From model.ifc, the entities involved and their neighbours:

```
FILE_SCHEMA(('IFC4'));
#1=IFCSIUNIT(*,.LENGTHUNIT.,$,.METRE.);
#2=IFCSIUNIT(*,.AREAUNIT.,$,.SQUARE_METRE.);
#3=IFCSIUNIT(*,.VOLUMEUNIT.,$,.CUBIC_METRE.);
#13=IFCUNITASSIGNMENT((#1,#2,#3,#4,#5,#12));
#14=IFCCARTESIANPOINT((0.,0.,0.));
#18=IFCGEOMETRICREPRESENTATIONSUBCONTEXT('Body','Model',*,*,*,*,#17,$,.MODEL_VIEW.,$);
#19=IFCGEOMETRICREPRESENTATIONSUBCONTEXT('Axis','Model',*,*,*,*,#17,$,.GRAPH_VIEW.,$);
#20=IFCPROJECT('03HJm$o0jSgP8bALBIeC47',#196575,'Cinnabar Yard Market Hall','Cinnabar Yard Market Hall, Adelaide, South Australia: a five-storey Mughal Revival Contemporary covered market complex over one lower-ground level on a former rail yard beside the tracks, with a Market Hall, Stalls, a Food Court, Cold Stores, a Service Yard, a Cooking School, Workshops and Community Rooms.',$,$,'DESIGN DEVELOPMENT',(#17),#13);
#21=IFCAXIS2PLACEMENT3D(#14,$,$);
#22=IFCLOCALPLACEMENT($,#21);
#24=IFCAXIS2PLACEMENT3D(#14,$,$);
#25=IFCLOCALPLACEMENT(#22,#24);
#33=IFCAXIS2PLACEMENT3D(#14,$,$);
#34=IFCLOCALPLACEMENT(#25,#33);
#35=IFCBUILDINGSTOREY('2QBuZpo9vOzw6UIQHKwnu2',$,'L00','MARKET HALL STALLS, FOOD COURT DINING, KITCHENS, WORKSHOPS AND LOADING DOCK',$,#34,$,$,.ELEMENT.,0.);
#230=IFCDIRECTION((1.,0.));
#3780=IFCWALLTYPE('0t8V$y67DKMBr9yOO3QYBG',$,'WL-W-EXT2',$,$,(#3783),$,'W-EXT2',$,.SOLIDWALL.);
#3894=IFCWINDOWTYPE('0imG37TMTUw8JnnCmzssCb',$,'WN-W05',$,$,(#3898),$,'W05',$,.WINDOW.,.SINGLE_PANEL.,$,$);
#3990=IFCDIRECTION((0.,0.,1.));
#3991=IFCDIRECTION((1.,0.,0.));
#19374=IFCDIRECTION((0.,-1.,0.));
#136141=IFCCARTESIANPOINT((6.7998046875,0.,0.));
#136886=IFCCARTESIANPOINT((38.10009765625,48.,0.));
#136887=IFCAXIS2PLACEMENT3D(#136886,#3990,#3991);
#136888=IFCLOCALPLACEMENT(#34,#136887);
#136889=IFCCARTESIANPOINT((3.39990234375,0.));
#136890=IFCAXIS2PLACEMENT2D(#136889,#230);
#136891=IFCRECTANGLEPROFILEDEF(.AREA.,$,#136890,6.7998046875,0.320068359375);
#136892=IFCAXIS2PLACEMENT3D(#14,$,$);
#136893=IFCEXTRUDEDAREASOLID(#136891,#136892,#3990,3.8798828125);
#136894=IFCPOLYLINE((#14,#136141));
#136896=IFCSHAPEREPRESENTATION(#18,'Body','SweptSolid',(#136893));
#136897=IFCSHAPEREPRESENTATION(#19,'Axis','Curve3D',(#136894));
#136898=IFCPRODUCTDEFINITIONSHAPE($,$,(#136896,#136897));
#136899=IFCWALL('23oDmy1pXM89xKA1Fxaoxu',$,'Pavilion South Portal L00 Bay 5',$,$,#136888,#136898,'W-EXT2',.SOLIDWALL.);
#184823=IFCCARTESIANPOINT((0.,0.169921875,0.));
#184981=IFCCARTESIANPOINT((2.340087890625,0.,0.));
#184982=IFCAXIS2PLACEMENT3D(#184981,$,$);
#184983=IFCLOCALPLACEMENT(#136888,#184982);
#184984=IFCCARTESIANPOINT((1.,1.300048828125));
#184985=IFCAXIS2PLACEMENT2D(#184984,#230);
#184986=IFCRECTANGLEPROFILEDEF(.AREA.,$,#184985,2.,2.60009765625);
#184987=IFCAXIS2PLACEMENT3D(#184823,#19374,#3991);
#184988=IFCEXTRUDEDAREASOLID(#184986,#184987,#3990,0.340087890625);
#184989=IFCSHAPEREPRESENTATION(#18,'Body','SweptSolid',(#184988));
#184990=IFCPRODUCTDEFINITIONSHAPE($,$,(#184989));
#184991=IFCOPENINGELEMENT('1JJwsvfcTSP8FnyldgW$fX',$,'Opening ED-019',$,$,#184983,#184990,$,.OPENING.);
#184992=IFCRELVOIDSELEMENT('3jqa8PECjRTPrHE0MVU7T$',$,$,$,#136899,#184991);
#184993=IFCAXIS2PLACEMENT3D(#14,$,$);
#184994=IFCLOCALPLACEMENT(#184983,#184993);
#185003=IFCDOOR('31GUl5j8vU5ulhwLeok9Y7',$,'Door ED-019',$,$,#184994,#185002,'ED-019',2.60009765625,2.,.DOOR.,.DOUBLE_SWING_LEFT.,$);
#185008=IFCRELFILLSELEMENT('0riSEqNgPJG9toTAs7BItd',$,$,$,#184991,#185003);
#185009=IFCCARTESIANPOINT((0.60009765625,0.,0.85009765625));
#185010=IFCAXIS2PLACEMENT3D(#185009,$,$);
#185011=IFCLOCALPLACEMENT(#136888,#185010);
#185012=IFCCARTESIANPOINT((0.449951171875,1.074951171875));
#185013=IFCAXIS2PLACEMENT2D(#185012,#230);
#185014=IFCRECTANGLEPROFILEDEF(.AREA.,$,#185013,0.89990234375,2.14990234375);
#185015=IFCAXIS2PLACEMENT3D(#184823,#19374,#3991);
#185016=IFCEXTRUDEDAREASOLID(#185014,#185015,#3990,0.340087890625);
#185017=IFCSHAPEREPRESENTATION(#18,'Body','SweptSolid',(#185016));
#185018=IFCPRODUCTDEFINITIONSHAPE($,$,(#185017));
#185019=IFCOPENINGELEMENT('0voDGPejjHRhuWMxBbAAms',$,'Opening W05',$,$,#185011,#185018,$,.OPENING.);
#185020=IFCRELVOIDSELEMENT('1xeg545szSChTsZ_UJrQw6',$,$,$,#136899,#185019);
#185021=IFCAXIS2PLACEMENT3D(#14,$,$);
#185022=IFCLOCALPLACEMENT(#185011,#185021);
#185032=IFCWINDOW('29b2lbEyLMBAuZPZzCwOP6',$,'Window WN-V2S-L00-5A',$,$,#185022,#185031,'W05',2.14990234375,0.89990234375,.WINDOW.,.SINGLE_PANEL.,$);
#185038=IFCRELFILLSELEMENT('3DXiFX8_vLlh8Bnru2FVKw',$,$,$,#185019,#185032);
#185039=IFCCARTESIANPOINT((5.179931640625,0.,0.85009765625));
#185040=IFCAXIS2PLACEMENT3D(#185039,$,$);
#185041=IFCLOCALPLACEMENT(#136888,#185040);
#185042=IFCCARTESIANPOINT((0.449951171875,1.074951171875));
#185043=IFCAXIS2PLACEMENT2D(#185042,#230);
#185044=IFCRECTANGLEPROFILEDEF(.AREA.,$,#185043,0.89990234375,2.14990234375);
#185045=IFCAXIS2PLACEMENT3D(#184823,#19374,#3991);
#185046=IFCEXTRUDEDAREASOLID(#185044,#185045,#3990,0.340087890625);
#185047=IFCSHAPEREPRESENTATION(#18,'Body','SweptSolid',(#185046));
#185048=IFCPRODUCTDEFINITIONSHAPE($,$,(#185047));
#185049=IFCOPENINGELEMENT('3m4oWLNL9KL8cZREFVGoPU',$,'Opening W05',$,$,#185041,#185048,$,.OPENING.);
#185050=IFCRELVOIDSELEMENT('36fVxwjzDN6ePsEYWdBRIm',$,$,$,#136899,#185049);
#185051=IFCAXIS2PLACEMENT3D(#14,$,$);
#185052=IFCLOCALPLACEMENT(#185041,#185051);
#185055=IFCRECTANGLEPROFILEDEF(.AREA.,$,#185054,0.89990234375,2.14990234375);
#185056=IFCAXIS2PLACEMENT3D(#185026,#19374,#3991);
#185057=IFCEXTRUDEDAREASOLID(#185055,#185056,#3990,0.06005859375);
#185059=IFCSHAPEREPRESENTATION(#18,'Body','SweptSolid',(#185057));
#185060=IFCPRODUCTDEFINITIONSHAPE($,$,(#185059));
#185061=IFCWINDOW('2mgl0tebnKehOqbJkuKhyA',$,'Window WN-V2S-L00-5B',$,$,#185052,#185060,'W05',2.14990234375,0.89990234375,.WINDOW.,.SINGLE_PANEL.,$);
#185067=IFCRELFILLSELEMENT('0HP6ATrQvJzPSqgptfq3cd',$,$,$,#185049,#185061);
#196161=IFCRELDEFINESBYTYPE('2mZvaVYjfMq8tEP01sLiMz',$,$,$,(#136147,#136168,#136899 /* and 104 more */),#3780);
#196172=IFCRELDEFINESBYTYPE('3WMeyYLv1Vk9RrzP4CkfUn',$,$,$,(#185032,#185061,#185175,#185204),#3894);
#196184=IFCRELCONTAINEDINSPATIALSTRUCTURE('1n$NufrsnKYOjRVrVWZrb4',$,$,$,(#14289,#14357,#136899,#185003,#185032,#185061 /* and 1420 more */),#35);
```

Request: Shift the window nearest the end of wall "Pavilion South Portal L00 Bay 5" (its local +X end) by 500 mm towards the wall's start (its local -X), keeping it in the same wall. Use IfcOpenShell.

```python
import ifcopenshell
import ifcopenshell.api.geometry
import ifcopenshell.util.placement
import ifcopenshell.util.unit

model = ifcopenshell.open("model.ifc")
unit_scale = ifcopenshell.util.unit.calculate_unit_scale(model)

window = model.by_id(185061)
opening = window.FillsVoids[0].RelatingOpeningElement
wall = opening.VoidsElements[0].RelatingBuildingElement

wall_matrix = ifcopenshell.util.placement.get_local_placement(wall.ObjectPlacement)
shift = wall_matrix[:3, 0] * -0.5 / unit_scale
before = ifcopenshell.util.placement.get_local_placement(window.ObjectPlacement)[:3, 3].copy()

# The window is placed relative to its opening, so it follows when the opening moves.
matrix = ifcopenshell.util.placement.get_local_placement(opening.ObjectPlacement)
matrix[:3, 3] += shift
ifcopenshell.api.geometry.edit_object_placement(
    model, product=opening, matrix=matrix, is_si=False, should_transform_children=True
)

after = ifcopenshell.util.placement.get_local_placement(window.ObjectPlacement)[:3, 3]
print("window moved by", (after - before).round(3) + 0.0)

model.write("model_updated.ifc")
```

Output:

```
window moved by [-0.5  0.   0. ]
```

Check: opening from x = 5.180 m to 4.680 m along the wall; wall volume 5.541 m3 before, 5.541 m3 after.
